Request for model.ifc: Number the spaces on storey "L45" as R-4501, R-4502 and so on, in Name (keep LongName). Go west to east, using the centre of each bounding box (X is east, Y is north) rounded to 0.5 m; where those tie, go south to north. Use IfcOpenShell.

First a look at what the model holds.

```python
import ifcopenshell
import ifcopenshell.util.element
import ifcopenshell.util.placement

model = ifcopenshell.open("model.ifc")
print(model.schema)
storey = next(s for s in model.by_type("IfcBuildingStorey") if s.Name == "L45")
spaces = [e for e in ifcopenshell.util.element.get_decomposition(storey) if e.is_a("IfcSpace")]
for e in sorted(spaces, key=lambda e: e.id()):
    origin = ifcopenshell.util.placement.get_local_placement(e.ObjectPlacement)[:3, 3]
    print(e.id(), e.Name, e.LongName, origin.round(2) + 0.0, sep=" | ")
```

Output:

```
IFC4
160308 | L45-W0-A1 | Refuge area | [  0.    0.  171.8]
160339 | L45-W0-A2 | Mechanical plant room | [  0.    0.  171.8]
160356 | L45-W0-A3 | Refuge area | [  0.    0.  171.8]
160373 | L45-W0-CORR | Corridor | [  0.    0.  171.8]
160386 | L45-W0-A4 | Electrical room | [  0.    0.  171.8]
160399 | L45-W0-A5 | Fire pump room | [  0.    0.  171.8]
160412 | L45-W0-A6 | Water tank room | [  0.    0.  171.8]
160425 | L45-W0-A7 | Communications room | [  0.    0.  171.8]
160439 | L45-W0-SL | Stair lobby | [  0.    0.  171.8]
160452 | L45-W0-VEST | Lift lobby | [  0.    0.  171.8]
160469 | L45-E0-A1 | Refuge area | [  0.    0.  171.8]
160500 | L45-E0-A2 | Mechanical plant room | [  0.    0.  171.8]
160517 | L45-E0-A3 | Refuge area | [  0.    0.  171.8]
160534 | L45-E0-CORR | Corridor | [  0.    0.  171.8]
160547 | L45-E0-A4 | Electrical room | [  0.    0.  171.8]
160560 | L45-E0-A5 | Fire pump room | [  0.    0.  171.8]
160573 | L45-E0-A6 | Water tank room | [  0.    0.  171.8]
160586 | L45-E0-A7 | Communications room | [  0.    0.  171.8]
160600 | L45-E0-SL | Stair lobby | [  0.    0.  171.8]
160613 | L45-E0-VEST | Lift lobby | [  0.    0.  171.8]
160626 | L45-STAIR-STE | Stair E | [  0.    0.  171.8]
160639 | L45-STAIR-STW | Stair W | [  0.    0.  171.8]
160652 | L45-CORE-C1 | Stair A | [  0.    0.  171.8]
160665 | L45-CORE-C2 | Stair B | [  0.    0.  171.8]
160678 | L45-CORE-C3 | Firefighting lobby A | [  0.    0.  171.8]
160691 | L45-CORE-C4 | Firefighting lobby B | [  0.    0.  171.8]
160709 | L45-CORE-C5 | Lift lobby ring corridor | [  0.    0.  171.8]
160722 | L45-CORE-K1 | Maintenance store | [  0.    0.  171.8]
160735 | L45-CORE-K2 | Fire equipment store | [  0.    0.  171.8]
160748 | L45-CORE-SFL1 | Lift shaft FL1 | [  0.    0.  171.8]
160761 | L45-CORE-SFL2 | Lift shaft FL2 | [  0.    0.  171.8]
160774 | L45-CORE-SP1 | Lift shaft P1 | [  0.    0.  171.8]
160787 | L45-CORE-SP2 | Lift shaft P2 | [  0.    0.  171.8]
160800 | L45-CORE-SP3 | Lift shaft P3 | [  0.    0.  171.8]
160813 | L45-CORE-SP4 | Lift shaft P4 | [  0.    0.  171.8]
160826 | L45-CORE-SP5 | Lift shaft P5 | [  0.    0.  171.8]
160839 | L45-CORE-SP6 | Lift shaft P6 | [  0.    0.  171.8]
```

```python
import ifcopenshell
import ifcopenshell.geom
import ifcopenshell.util.element
import ifcopenshell.util.shape

model = ifcopenshell.open("model.ifc")
settings = ifcopenshell.geom.settings()
settings.set("use-world-coords", True)


def centre(element):
    shape = ifcopenshell.geom.create_shape(settings, element)
    return ifcopenshell.util.shape.get_bbox_centroid(shape.geometry)


storey = next(s for s in model.by_type("IfcBuildingStorey") if s.Name == "L45")
spaces = [e for e in ifcopenshell.util.element.get_decomposition(storey) if e.is_a("IfcSpace")]

# Insertion points can sit at a corner or the storey origin, so sort by the geometry (in metres).
centres = {e: centre(e) for e in spaces}
spaces.sort(key=lambda e: (round(centres[e][0] / 0.5), centres[e][1]))

for i, e in enumerate(spaces, start=1):
    number = f"R-45{i:02d}"
    e.Name = number
    print(e.id(), number)

model.write("model_updated.ifc")
```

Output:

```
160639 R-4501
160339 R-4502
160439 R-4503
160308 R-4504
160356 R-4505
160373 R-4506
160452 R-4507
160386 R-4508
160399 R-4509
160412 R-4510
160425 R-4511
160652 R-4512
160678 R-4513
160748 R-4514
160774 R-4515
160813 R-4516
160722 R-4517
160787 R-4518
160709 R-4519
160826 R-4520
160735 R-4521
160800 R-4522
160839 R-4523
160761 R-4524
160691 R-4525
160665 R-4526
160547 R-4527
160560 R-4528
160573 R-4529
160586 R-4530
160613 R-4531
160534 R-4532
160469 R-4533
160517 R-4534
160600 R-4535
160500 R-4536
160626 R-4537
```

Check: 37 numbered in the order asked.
